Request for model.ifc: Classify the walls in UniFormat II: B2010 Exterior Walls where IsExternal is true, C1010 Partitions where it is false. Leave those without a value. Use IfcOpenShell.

First a look at what the model holds.

```python
import ifcopenshell
import ifcopenshell.util.element

model = ifcopenshell.open("model.ifc")
print(model.schema)
print("classifications:", [c.Name for c in model.by_type("IfcClassification")])
values = [ifcopenshell.util.element.get_pset(e, "Pset_WallCommon", "IsExternal") for e in model.by_type("IfcWall")]
for value in (True, False, None):
    print("IsExternal", value, values.count(value))
```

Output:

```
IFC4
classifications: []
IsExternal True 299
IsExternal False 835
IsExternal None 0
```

```python
import ifcopenshell
import ifcopenshell.api.classification
import ifcopenshell.util.element

model = ifcopenshell.open("model.ifc")

system = ifcopenshell.api.classification.add_classification(model, classification="UniFormat II")

walls = model.by_type("IfcWall")
external = {e: ifcopenshell.util.element.get_pset(e, "Pset_WallCommon", "IsExternal") for e in walls}
for flag, code, name in ((True, "B2010", "Exterior Walls"), (False, "C1010", "Partitions")):
    products = [e for e in walls if external[e] is flag]
    ifcopenshell.api.classification.add_reference(
        model, products=products, classification=system, identification=code, name=name
    )
    print(code, len(products))

model.write("model_v2.ifc")
```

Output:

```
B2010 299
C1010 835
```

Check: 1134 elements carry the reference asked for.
